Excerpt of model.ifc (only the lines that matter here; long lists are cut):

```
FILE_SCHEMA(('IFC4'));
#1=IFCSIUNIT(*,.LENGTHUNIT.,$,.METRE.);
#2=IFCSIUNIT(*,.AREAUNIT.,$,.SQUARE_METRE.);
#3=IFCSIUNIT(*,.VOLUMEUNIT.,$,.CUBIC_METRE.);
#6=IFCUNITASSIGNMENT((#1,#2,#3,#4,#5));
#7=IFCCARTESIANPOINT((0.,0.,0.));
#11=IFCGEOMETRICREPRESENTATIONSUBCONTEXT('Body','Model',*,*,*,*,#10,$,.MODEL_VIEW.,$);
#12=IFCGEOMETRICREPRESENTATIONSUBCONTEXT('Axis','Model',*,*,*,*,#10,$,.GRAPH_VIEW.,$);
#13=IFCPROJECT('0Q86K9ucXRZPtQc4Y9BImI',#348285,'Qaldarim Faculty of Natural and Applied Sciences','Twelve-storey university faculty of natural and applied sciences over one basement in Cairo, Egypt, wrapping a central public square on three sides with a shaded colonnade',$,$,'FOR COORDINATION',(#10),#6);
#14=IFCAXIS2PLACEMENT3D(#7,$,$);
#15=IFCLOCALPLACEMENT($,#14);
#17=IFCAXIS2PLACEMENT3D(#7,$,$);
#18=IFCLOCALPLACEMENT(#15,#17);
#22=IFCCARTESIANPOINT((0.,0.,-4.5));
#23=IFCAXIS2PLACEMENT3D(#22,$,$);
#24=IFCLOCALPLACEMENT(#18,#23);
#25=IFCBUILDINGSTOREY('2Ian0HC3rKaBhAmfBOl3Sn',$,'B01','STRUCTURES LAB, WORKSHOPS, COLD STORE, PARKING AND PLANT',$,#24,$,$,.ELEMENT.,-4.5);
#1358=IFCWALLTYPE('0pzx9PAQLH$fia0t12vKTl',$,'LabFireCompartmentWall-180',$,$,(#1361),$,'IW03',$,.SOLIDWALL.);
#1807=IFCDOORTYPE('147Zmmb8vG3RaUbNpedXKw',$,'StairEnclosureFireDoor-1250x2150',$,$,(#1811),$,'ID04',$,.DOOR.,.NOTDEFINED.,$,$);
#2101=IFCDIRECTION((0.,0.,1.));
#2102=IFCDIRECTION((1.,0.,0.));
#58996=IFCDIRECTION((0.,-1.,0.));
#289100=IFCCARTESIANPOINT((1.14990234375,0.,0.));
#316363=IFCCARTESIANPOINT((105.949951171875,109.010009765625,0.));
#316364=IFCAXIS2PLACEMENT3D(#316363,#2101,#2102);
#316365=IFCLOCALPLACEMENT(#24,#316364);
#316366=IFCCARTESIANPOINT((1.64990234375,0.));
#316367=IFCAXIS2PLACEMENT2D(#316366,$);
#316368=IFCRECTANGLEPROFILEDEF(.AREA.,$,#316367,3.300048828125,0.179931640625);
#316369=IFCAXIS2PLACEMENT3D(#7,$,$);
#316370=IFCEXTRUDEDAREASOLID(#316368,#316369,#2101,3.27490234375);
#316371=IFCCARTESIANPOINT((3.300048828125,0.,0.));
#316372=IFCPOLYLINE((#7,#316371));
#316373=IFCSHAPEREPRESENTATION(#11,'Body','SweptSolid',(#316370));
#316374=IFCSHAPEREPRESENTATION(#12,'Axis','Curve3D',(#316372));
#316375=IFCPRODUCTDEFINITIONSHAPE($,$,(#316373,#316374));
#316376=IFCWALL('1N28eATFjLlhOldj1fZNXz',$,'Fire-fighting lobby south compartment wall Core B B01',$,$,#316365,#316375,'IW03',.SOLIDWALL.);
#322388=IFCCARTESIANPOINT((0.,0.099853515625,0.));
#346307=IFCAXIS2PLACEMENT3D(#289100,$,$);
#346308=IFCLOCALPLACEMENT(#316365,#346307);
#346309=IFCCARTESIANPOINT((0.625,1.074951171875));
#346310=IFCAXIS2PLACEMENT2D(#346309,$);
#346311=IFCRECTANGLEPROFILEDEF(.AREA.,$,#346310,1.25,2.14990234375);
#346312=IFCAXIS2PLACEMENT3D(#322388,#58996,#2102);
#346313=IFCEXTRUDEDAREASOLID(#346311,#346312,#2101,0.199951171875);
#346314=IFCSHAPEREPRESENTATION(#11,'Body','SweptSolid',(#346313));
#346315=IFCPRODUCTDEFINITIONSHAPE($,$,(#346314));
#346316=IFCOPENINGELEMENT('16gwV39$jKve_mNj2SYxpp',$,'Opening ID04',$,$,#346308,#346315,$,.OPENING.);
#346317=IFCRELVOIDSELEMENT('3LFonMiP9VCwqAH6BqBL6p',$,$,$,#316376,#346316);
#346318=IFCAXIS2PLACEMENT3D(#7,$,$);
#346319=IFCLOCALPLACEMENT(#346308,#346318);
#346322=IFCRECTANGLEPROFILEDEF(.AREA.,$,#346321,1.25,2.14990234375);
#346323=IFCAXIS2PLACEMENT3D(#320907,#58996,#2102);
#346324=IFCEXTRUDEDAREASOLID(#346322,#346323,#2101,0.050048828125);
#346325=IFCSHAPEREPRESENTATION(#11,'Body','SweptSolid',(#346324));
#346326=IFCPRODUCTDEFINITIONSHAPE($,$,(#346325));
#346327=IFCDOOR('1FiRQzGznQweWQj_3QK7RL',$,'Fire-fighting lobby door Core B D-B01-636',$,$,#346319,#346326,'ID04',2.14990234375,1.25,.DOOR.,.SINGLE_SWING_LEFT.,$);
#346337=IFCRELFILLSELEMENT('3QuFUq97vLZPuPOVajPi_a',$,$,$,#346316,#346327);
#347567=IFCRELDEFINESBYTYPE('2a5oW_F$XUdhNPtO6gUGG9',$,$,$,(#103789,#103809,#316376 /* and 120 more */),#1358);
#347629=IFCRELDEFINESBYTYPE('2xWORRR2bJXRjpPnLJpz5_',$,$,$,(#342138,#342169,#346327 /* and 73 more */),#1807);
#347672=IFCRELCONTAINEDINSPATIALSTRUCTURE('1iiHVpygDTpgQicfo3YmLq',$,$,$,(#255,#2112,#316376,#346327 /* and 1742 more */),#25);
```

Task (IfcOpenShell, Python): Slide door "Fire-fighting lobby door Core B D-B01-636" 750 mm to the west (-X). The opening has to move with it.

```python
import ifcopenshell
import ifcopenshell.api.geometry
import ifcopenshell.util.placement

model = ifcopenshell.open("model.ifc")

door = model.by_guid("1FiRQzGznQweWQj_3QK7RL")
opening = door.FillsVoids[0].RelatingOpeningElement
wall = opening.VoidsElements[0].RelatingBuildingElement

wall_matrix = ifcopenshell.util.placement.get_local_placement(wall.ObjectPlacement)
shift = wall_matrix[:3, 0] * -0.75
before = ifcopenshell.util.placement.get_local_placement(door.ObjectPlacement)[:3, 3].copy()

# The door is placed relative to its opening, so it follows when the opening moves.
matrix = ifcopenshell.util.placement.get_local_placement(opening.ObjectPlacement)
matrix[:3, 3] += shift
ifcopenshell.api.geometry.edit_object_placement(
    model, product=opening, matrix=matrix, is_si=False, should_transform_children=True
)

after = ifcopenshell.util.placement.get_local_placement(door.ObjectPlacement)[:3, 3]
print("door moved by", (after - before).round(3) + 0.0)

model.write("model_edited.ifc")
```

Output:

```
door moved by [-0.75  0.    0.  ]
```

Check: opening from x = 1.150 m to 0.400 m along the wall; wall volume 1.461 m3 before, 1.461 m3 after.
